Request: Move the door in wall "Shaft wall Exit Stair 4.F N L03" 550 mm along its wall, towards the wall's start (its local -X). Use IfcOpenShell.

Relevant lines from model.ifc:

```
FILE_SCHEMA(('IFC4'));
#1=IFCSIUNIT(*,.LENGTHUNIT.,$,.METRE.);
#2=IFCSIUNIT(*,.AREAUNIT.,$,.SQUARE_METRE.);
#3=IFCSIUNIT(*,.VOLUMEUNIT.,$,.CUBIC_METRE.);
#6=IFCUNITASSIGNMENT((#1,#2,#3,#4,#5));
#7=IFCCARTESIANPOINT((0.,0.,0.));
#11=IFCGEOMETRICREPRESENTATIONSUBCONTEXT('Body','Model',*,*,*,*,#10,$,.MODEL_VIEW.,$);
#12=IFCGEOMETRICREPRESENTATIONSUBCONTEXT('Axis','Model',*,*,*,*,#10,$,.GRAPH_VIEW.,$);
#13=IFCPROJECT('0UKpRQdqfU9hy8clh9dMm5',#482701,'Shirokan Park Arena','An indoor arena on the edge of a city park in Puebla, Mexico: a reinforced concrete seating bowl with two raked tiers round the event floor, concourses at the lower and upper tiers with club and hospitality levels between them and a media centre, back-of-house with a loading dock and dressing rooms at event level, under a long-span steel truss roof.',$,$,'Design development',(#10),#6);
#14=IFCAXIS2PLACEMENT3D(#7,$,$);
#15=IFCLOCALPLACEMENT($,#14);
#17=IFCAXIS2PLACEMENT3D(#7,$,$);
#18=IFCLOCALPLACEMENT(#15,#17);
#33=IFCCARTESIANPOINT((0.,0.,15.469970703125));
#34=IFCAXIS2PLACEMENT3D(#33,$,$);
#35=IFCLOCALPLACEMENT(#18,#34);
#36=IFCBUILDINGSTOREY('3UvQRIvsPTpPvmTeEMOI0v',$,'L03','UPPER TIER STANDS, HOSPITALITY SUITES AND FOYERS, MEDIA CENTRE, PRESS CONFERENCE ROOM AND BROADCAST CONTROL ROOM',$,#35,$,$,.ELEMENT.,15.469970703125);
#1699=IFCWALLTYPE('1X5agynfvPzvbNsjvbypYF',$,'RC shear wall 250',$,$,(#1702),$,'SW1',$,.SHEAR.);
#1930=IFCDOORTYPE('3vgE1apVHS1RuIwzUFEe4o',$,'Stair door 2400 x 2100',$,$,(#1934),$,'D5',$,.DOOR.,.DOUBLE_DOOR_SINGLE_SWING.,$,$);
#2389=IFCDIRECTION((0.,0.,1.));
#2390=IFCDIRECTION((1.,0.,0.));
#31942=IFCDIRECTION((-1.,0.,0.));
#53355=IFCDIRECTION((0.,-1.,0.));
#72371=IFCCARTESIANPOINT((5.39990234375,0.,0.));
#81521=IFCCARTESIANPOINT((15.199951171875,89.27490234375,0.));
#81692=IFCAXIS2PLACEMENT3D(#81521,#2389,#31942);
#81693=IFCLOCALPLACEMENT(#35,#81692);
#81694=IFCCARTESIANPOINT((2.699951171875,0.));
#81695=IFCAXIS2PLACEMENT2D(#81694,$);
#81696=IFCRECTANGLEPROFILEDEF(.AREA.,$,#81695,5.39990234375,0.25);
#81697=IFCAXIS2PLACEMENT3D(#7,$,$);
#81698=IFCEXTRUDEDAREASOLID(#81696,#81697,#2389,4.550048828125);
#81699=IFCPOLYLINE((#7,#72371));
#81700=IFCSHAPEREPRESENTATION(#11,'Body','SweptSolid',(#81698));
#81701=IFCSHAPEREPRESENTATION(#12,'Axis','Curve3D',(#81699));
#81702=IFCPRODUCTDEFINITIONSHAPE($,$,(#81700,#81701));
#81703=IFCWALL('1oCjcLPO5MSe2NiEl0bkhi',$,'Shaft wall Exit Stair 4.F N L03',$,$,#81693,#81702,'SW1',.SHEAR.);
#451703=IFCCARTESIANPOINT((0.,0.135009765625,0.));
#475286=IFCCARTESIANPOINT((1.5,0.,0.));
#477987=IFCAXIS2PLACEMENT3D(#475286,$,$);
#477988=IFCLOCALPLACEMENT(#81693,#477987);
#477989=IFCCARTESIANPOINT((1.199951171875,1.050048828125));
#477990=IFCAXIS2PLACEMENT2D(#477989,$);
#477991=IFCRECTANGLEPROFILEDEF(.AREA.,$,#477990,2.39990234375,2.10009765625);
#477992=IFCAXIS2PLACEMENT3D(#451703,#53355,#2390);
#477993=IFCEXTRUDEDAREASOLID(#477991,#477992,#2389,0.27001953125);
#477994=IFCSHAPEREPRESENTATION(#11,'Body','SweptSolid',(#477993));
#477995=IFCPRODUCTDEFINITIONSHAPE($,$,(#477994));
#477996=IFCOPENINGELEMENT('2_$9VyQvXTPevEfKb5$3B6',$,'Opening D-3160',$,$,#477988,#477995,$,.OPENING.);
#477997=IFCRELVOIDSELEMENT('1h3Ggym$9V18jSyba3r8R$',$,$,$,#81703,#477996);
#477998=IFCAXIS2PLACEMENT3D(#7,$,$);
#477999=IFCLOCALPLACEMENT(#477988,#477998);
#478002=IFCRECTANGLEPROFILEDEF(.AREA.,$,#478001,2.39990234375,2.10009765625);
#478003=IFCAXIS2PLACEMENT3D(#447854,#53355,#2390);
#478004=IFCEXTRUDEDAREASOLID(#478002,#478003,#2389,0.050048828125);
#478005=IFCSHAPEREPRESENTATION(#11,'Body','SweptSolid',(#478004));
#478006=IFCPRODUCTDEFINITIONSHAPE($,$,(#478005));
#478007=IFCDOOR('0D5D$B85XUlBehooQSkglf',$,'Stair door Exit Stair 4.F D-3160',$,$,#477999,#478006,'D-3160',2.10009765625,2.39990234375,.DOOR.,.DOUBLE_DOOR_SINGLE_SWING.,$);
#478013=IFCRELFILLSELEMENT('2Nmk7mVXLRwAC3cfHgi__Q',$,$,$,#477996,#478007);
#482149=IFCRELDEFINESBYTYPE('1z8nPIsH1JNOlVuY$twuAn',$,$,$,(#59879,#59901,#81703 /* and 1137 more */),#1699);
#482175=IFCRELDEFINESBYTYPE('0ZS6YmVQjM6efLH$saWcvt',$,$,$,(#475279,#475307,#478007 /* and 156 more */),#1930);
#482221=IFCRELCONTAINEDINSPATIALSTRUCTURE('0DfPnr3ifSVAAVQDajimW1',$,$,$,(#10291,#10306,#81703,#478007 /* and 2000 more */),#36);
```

```python
import ifcopenshell
import ifcopenshell.api.geometry
import ifcopenshell.util.placement

model = ifcopenshell.open("model.ifc")

door = model.by_guid("0D5D$B85XUlBehooQSkglf")
opening = door.FillsVoids[0].RelatingOpeningElement
wall = opening.VoidsElements[0].RelatingBuildingElement

wall_matrix = ifcopenshell.util.placement.get_local_placement(wall.ObjectPlacement)
shift = wall_matrix[:3, 0] * -0.55
before = ifcopenshell.util.placement.get_local_placement(door.ObjectPlacement)[:3, 3].copy()

# The door is placed relative to its opening, so it follows when the opening moves.
matrix = ifcopenshell.util.placement.get_local_placement(opening.ObjectPlacement)
matrix[:3, 3] += shift
ifcopenshell.api.geometry.edit_object_placement(
    model, product=opening, matrix=matrix, is_si=False, should_transform_children=True
)

after = ifcopenshell.util.placement.get_local_placement(door.ObjectPlacement)[:3, 3]
print("door moved by", (after - before).round(3) + 0.0)

model.write("model_updated.ifc")
```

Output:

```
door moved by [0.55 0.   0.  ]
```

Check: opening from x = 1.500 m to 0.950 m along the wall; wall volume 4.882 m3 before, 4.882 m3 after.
